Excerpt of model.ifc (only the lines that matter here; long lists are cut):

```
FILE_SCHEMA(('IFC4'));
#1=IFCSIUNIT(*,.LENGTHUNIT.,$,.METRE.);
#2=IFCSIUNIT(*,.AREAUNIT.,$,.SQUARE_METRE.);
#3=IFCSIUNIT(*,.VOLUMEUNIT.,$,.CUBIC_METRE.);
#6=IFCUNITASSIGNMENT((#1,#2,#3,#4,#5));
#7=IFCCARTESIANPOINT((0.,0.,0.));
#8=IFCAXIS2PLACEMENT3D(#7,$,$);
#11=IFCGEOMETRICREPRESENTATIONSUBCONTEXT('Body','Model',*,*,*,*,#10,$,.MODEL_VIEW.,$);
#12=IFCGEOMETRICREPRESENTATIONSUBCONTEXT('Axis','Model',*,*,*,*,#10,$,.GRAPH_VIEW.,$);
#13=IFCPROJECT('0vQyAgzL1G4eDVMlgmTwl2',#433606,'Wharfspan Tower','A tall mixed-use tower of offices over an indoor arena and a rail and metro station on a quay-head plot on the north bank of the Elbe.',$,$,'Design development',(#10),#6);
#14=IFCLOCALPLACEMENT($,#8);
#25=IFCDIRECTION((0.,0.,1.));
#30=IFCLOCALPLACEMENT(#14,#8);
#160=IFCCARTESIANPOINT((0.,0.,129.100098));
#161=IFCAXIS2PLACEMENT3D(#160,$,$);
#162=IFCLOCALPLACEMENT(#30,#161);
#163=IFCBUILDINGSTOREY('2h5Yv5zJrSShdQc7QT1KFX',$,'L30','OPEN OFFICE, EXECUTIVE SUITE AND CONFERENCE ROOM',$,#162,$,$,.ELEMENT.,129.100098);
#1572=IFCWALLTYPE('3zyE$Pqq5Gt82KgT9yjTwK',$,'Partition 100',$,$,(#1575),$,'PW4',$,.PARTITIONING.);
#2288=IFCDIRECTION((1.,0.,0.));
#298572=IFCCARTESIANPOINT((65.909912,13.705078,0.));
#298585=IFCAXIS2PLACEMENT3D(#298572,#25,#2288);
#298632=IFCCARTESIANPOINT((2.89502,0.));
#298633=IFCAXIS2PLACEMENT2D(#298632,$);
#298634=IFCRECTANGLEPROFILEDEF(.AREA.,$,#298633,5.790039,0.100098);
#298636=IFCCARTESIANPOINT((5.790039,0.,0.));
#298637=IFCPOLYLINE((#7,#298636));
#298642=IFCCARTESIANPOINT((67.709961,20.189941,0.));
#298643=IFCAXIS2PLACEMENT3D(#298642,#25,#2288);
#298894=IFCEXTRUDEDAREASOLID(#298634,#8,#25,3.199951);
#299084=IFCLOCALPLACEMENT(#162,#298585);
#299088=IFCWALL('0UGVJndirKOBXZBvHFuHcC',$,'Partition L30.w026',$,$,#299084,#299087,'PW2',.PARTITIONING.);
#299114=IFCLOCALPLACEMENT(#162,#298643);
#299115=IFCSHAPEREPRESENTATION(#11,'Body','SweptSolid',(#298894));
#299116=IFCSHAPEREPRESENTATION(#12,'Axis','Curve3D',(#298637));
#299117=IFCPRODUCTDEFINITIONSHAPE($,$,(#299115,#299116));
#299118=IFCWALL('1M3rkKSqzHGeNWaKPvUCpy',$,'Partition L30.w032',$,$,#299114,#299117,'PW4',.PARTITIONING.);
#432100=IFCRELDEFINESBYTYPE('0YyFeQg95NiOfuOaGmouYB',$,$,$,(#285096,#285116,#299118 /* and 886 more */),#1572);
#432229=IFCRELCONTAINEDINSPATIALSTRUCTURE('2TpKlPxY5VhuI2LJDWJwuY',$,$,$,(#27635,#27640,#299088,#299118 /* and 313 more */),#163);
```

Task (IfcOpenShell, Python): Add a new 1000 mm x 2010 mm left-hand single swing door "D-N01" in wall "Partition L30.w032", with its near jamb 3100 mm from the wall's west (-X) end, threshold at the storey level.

```python
import numpy as np
import ifcopenshell
import ifcopenshell.api.feature
import ifcopenshell.api.geometry
import ifcopenshell.api.root
import ifcopenshell.api.spatial
import ifcopenshell.geom
import ifcopenshell.util.element
import ifcopenshell.util.placement
import ifcopenshell.util.representation
import ifcopenshell.util.shape
import ifcopenshell.util.unit

model = ifcopenshell.open("model.ifc")
unit_scale = ifcopenshell.util.unit.calculate_unit_scale(model)
settings = ifcopenshell.geom.settings()


def volume(element):
    """Net volume in cubic metres, openings subtracted."""
    shape = ifcopenshell.geom.create_shape(settings, element)
    return ifcopenshell.util.shape.get_volume(shape.geometry)


wall = model.by_guid("1M3rkKSqzHGeNWaKPvUCpy")
storey = ifcopenshell.util.element.get_container(wall, ifc_class="IfcBuildingStorey")
context = ifcopenshell.util.representation.get_context(model, "Model", "Body", "MODEL_VIEW")
before = volume(wall)

width, height, from_end, sill = 1, 2.01, 3.1, 0.0  # metres

# The wall runs along its own X axis, and the end named is its -X end.
wall_shape = ifcopenshell.geom.create_shape(settings, wall)
x, y, z = ifcopenshell.util.shape.get_vertices(wall_shape.geometry).T
start = x.min() + from_end
face, thickness = float(y.min()), float(y.max() - y.min())
wall_matrix = ifcopenshell.util.placement.get_local_placement(wall.ObjectPlacement)
level = ifcopenshell.util.placement.get_local_placement(storey.ObjectPlacement)[2, 3]


def in_wall(x, y):
    """Placement at x, y metres in the wall's axes, at sill height."""
    matrix = wall_matrix.copy()
    matrix[:, 3] = wall_matrix @ np.array([x / unit_scale, y / unit_scale, 0.0, 1.0])
    matrix[2, 3] = level + sill / unit_scale
    return matrix


# Opening: a box that overshoots both wall faces by 50 mm.
opening = ifcopenshell.api.root.create_entity(model, ifc_class="IfcOpeningElement", predefined_type="OPENING")
box = ifcopenshell.api.geometry.add_wall_representation(
    model, context=context, length=width, height=height, thickness=thickness + 0.1
)
ifcopenshell.api.geometry.assign_representation(model, product=opening, representation=box)
ifcopenshell.api.geometry.edit_object_placement(model, product=opening, matrix=in_wall(start, face - 0.05), is_si=False)
ifcopenshell.api.feature.add_feature(model, feature=opening, element=wall)

door = ifcopenshell.api.root.create_entity(model, ifc_class="IfcDoor", name="D-N01", predefined_type="DOOR")
door.OverallWidth, door.OverallHeight = width / unit_scale, height / unit_scale
door.OperationType = "SINGLE_SWING_LEFT"
body = ifcopenshell.api.geometry.add_door_representation(
    model,
    context=context,
    overall_width=door.OverallWidth,
    overall_height=door.OverallHeight,
    operation_type="SINGLE_SWING_LEFT",
    lining_properties={"LiningDepth": thickness / unit_scale, "ThresholdDepth": thickness / unit_scale},
)
ifcopenshell.api.geometry.assign_representation(model, product=door, representation=body)
ifcopenshell.api.spatial.assign_container(model, products=[door], relating_structure=storey)
ifcopenshell.api.feature.add_filling(model, opening=opening, element=door)

# The lining spans the wall, so the door starts at the wall face.
ifcopenshell.api.geometry.edit_object_placement(model, product=door, matrix=in_wall(start, face), is_si=False)

after = volume(wall)

print(f"wall volume {before:.3f} -> {after:.3f} m3")

model.write("model_updated.ifc")
```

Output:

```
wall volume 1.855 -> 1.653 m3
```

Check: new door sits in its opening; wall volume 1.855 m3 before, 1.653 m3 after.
